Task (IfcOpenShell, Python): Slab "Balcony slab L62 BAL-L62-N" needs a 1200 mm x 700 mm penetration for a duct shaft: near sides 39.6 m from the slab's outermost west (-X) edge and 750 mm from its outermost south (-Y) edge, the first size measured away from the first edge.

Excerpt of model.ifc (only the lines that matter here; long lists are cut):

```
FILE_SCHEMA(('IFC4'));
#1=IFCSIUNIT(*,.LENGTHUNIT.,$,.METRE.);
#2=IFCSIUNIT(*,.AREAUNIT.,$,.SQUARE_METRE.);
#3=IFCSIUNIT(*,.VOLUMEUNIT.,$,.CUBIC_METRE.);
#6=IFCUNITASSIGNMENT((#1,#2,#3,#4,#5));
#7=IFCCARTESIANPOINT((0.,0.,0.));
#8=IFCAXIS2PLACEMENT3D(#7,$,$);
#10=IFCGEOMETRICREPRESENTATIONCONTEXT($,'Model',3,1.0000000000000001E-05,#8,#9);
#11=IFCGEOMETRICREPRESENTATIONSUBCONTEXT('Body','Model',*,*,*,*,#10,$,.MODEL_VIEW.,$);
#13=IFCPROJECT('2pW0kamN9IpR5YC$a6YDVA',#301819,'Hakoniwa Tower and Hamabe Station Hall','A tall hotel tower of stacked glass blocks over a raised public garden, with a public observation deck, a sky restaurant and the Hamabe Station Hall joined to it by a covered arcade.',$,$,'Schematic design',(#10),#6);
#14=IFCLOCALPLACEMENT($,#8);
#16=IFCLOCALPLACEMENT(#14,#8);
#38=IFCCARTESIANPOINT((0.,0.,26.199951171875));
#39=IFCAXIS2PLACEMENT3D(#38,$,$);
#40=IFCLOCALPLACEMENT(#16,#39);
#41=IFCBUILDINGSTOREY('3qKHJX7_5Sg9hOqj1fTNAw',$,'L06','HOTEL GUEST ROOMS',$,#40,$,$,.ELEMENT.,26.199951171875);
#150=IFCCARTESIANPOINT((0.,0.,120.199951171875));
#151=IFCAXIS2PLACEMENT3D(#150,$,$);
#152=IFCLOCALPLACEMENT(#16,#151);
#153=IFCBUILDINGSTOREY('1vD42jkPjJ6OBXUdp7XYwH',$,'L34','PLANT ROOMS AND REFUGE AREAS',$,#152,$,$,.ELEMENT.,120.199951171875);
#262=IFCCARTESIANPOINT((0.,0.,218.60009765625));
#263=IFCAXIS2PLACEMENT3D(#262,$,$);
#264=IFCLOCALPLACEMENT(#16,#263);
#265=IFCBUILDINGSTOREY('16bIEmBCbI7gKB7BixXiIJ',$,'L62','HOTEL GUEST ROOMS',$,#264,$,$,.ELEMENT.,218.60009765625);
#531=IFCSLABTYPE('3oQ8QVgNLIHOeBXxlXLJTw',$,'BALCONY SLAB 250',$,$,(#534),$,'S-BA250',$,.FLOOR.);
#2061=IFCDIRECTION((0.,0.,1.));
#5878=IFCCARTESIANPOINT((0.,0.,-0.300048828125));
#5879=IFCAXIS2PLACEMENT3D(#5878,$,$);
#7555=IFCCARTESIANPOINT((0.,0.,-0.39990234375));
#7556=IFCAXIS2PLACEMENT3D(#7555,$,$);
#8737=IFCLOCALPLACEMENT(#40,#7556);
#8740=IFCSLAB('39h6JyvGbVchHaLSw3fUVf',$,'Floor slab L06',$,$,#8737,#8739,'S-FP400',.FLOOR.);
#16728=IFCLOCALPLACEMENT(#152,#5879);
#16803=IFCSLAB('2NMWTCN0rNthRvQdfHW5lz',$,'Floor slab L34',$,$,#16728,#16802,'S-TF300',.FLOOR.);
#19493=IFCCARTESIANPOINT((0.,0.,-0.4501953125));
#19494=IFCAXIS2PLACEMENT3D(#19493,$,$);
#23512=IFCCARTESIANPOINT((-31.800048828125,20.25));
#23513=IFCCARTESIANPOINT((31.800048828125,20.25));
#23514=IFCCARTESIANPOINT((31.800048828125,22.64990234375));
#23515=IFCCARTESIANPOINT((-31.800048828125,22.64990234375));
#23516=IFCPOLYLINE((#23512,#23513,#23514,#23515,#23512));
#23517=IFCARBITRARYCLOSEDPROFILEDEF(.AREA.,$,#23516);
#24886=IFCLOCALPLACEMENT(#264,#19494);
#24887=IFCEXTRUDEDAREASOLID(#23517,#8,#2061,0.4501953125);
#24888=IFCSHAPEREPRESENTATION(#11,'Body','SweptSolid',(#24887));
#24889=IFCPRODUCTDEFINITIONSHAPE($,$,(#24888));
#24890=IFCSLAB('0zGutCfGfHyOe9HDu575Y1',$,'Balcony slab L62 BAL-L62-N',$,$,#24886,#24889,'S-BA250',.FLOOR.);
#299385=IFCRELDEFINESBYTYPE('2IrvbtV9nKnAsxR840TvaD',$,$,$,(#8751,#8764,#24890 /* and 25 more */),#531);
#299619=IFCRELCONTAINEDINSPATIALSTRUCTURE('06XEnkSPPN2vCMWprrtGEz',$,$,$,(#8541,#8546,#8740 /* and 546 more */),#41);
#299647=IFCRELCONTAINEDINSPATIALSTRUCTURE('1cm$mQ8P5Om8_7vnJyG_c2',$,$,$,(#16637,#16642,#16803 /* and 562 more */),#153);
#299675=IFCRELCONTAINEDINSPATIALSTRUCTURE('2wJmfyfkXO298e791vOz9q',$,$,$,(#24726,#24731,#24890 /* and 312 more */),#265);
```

```python
import numpy as np
import ifcopenshell
import ifcopenshell.api.feature
import ifcopenshell.api.geometry
import ifcopenshell.api.root
import ifcopenshell.geom
import ifcopenshell.util.placement
import ifcopenshell.util.representation
import ifcopenshell.util.shape
import ifcopenshell.util.unit

model = ifcopenshell.open("model.ifc")
unit_scale = ifcopenshell.util.unit.calculate_unit_scale(model)
settings = ifcopenshell.geom.settings()


def volume(element):
    """Net volume in cubic metres, openings subtracted."""
    shape = ifcopenshell.geom.create_shape(settings, element)
    return ifcopenshell.util.shape.get_volume(shape.geometry)


slab = model.by_id(24890)
before = volume(slab)

# Extent in the slab's own axes, in metres. The edges named are its -X and -Y sides.
slab_shape = ifcopenshell.geom.create_shape(settings, slab)
vertices = ifcopenshell.util.shape.get_vertices(slab_shape.geometry)
x_min, y_min, bottom = vertices.min(axis=0)
top = vertices[:, 2].max()

opening = ifcopenshell.api.root.create_entity(model, ifc_class="IfcOpeningElement", name="Duct shaft opening", predefined_type="OPENING")
context = ifcopenshell.util.representation.get_context(model, "Model", "Body", "MODEL_VIEW")
width, depth = 1.2, 0.7
outline = [(0.0, 0.0), (width, 0.0), (width, depth), (0.0, depth), (0.0, 0.0)]
# Overshoot both faces by 50 mm so the cut is clean.
shape = ifcopenshell.api.geometry.add_slab_representation(
    model, context=context, depth=top - bottom + 0.1, polyline=outline
)
ifcopenshell.api.geometry.assign_representation(model, product=opening, representation=shape)

matrix = ifcopenshell.util.placement.get_local_placement(slab.ObjectPlacement)
matrix[:, 3] = matrix @ np.append(np.array([x_min + 39.6, y_min + 0.75, bottom - 0.05]) / unit_scale, 1.0)
ifcopenshell.api.geometry.edit_object_placement(model, product=opening, matrix=matrix, is_si=False)
ifcopenshell.api.feature.add_feature(model, feature=opening, element=slab)

after = volume(slab)

print(f"slab volume {before:.3f} -> {after:.3f} m3")

model.write("model-out.ifc")
```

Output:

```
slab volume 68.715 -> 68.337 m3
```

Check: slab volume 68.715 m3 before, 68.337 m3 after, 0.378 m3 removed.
